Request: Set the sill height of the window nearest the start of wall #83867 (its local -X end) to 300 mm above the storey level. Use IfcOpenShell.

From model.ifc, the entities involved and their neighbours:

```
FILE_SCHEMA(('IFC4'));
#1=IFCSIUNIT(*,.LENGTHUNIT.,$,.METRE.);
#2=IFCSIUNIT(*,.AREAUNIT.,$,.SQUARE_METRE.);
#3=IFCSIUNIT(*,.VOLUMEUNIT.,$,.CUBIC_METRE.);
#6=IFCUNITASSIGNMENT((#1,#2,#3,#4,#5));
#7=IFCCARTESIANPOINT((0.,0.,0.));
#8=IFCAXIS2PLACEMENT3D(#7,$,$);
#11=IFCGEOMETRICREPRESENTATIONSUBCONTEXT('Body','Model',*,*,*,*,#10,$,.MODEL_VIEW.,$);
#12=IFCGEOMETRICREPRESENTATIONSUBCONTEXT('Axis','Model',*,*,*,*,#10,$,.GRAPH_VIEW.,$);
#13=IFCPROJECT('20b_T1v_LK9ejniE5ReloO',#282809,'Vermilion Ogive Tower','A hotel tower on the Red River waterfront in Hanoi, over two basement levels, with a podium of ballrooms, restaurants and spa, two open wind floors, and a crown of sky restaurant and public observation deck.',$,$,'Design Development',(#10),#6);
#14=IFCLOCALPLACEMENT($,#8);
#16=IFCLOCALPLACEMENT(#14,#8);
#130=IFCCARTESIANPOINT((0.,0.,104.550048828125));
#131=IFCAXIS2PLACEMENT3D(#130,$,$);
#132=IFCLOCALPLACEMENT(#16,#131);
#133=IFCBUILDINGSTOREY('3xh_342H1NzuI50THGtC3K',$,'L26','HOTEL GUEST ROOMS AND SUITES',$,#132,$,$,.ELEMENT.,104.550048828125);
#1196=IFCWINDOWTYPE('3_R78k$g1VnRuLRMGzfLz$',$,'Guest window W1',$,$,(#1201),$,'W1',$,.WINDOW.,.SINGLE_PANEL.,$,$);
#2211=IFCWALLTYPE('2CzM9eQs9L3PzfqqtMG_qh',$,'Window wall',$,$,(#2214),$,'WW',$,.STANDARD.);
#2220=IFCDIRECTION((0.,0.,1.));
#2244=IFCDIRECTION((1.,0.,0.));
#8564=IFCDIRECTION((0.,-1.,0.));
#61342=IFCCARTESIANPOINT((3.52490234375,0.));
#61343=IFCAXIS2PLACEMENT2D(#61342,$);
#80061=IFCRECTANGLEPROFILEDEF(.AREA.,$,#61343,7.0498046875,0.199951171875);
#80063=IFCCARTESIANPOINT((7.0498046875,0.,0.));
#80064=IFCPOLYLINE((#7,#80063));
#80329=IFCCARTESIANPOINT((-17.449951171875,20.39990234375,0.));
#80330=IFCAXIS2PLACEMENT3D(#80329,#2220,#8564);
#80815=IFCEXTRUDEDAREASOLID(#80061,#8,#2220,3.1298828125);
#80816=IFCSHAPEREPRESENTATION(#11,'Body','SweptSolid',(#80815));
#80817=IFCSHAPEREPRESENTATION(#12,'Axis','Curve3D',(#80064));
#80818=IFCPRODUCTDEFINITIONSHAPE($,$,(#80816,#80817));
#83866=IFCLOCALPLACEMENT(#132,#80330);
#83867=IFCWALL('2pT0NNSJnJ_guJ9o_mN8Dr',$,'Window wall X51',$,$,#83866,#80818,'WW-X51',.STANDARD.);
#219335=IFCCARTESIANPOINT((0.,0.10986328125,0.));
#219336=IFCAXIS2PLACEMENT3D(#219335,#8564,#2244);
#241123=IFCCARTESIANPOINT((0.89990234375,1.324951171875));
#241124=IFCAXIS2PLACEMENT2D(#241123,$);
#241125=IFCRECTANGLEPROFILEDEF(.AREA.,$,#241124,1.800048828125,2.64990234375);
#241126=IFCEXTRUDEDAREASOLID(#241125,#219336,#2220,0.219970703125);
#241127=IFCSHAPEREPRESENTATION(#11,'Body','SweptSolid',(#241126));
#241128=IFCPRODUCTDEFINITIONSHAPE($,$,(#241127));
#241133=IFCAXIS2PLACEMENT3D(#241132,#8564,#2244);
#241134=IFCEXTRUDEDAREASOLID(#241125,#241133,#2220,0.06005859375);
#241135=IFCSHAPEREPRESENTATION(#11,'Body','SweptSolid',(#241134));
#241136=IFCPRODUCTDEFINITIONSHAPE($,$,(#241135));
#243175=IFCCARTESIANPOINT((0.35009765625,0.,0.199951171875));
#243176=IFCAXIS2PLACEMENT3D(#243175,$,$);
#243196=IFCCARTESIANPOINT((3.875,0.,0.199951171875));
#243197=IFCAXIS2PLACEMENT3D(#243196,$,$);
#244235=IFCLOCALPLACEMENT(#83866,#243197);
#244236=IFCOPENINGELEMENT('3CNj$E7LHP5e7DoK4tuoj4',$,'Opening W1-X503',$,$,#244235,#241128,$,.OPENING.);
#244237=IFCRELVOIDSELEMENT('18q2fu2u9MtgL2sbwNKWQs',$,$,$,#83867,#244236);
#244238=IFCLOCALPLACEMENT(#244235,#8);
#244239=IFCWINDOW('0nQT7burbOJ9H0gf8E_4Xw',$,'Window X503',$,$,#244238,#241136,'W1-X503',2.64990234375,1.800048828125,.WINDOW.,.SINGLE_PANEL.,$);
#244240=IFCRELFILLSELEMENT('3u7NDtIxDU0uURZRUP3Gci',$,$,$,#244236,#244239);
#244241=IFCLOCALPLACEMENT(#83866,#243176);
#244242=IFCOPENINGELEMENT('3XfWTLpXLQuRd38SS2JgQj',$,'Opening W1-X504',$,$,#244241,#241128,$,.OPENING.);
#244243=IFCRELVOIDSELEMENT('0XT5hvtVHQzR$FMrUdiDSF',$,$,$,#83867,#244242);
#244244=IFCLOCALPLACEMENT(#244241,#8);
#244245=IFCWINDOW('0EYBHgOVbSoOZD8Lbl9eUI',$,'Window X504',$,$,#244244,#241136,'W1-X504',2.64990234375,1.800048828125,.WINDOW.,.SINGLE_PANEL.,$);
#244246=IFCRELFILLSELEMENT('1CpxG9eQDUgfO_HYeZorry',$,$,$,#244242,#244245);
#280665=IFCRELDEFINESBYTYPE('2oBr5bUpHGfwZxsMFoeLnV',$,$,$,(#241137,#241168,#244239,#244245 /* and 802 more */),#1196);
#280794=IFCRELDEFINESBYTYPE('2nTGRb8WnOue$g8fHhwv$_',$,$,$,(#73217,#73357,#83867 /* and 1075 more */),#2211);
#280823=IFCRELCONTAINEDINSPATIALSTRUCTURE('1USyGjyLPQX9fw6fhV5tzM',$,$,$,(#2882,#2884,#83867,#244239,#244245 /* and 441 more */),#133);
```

```python
import numpy as np
import ifcopenshell
import ifcopenshell.api.geometry
import ifcopenshell.geom
import ifcopenshell.util.element
import ifcopenshell.util.placement
import ifcopenshell.util.shape
import ifcopenshell.util.unit

model = ifcopenshell.open("model.ifc")
unit_scale = ifcopenshell.util.unit.calculate_unit_scale(model)

window = model.by_id(244245)
opening = window.FillsVoids[0].RelatingOpeningElement
storey = ifcopenshell.util.element.get_container(window, ifc_class="IfcBuildingStorey")
level = ifcopenshell.util.placement.get_local_placement(storey.ObjectPlacement)[2, 3]

# The opening's origin need not be at the sill, so measure its lowest point.
shape = ifcopenshell.geom.create_shape(ifcopenshell.geom.settings(), opening)
bottom = ifcopenshell.util.shape.get_shape_bottom_elevation(shape, shape.geometry) / unit_scale
dz = level + 0.3 - bottom

shift = np.array([0.0, 0.0, dz])
# The window is placed relative to its opening, so it follows when the opening moves.
matrix = ifcopenshell.util.placement.get_local_placement(opening.ObjectPlacement)
matrix[:3, 3] += shift
ifcopenshell.api.geometry.edit_object_placement(
    model, product=opening, matrix=matrix, is_si=False, should_transform_children=True
)

print(f"moved by {dz * unit_scale:+.3f} m")

model.write("model_rev.ifc")
```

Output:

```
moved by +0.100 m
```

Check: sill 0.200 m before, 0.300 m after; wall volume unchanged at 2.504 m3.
